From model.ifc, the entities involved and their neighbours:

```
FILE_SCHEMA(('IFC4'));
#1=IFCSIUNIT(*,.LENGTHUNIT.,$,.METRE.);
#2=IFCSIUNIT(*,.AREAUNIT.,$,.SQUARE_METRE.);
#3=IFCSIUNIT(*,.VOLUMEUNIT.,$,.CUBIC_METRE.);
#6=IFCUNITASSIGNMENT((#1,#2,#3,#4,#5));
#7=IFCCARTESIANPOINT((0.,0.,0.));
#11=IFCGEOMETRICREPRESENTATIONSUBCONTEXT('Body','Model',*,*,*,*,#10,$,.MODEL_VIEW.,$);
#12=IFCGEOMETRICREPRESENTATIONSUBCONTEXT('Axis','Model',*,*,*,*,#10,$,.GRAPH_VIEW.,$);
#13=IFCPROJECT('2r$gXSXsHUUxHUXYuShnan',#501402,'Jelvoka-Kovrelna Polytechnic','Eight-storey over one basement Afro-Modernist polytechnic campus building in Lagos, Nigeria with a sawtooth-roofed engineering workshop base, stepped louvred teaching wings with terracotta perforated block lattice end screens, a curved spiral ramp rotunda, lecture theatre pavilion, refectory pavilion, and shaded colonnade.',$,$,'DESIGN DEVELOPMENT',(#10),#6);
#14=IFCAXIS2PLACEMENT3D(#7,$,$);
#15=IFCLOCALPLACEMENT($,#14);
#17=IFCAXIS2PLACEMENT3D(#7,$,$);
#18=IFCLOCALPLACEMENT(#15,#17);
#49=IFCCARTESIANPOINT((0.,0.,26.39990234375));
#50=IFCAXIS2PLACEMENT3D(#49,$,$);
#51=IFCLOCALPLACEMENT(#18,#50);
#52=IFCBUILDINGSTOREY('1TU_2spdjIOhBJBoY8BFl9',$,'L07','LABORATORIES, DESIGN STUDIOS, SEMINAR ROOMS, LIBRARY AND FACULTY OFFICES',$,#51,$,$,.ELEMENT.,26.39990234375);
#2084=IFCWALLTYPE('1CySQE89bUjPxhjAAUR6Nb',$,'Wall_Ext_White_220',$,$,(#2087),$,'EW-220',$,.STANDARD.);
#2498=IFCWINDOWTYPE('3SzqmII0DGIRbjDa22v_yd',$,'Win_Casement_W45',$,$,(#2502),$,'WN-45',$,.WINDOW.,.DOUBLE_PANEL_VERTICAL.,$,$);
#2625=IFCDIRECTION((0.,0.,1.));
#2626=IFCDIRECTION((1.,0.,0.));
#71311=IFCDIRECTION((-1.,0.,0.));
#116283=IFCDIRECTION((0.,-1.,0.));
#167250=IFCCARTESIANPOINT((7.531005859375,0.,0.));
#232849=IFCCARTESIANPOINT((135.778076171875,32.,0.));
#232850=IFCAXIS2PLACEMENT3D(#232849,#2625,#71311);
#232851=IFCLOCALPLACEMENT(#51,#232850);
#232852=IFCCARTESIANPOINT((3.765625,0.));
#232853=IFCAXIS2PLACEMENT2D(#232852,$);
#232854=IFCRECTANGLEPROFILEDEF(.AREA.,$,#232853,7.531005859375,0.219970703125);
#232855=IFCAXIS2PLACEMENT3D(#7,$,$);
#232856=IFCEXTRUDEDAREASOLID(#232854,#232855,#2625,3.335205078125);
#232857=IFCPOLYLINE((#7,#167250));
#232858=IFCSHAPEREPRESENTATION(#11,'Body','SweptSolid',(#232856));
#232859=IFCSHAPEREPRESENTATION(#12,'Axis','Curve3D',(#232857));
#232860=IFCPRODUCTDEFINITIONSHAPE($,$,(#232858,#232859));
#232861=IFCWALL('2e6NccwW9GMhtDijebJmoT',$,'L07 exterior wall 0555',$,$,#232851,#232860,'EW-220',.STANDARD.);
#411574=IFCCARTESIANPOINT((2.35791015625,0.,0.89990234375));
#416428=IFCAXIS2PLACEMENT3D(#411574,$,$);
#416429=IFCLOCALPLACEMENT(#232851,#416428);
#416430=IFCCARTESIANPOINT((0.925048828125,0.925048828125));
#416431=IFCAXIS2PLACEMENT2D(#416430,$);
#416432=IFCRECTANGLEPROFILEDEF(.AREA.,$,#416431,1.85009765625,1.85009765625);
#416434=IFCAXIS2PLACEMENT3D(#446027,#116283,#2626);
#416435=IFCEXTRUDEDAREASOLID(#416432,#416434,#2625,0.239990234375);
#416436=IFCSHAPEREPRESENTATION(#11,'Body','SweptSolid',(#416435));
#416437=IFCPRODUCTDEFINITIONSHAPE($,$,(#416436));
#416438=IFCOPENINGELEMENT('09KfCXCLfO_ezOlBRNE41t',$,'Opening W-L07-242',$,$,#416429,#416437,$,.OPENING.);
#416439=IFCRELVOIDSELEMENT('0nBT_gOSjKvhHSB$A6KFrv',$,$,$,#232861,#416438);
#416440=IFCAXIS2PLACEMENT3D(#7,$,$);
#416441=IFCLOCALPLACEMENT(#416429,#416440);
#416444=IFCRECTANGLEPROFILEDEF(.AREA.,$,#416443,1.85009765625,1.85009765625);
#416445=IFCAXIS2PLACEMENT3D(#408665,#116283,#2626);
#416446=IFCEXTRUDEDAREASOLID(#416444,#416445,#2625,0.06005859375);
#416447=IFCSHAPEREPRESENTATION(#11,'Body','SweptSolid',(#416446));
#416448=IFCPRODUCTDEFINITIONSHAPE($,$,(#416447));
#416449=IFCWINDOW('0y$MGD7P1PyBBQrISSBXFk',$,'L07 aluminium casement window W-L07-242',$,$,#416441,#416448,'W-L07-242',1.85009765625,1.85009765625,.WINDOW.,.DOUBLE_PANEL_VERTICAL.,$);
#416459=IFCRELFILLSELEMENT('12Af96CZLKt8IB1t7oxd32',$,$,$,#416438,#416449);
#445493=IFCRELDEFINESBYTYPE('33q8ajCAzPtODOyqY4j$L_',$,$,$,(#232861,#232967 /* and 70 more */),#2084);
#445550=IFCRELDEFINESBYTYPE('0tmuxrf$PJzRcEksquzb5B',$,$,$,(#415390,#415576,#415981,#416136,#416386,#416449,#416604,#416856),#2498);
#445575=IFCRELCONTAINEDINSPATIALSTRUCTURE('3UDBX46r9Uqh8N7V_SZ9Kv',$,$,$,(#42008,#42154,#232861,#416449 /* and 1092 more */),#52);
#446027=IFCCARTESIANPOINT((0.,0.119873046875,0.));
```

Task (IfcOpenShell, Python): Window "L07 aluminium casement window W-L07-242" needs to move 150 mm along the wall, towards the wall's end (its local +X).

```python
import ifcopenshell
import ifcopenshell.api.geometry
import ifcopenshell.util.placement
import ifcopenshell.util.unit

model = ifcopenshell.open("model.ifc")
unit_scale = ifcopenshell.util.unit.calculate_unit_scale(model)

window = model.by_guid("0y$MGD7P1PyBBQrISSBXFk")
opening = window.FillsVoids[0].RelatingOpeningElement
wall = opening.VoidsElements[0].RelatingBuildingElement

wall_matrix = ifcopenshell.util.placement.get_local_placement(wall.ObjectPlacement)
shift = wall_matrix[:3, 0] * 0.15 / unit_scale
before = ifcopenshell.util.placement.get_local_placement(window.ObjectPlacement)[:3, 3].copy()

# The window is placed relative to its opening, so it follows when the opening moves.
matrix = ifcopenshell.util.placement.get_local_placement(opening.ObjectPlacement)
matrix[:3, 3] += shift
ifcopenshell.api.geometry.edit_object_placement(
    model, product=opening, matrix=matrix, is_si=False, should_transform_children=True
)

after = ifcopenshell.util.placement.get_local_placement(window.ObjectPlacement)[:3, 3]
print("window moved by", (after - before).round(3) + 0.0)

model.write("model_updated.ifc")
```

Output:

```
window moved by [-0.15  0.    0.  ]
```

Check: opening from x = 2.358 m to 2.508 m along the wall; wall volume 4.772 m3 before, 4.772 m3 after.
